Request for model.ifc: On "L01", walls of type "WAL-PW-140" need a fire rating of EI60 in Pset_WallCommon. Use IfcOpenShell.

First a look at what the model holds.

```python
import ifcopenshell
import ifcopenshell.util.element

model = ifcopenshell.open("model.ifc")
print(model.schema)
storey = next(s for s in model.by_type("IfcBuildingStorey") if s.Name == "L01")
walls = [e for e in ifcopenshell.util.element.get_decomposition(storey) if e.is_a("IfcWall")]
seen = {}
for e in walls:
    element_type = ifcopenshell.util.element.get_type(e)
    key = (element_type.Name if element_type != e and element_type else None, ifcopenshell.util.element.get_pset(e, "Pset_WallCommon", "FireRating"))
    seen[key] = seen.get(key, 0) + 1
for (name, value), count in sorted(seen.items(), key=str):
    print(count, "x", name, "|", value)
```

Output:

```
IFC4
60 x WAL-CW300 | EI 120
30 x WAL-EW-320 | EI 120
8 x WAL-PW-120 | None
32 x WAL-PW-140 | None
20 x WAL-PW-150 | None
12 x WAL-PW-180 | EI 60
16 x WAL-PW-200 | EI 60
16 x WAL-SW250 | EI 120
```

```python
import ifcopenshell
import ifcopenshell.api.pset
import ifcopenshell.util.element

model = ifcopenshell.open("model.ifc")

storey = next(s for s in model.by_type("IfcBuildingStorey") if s.Name == "L01")
walls = [e for e in ifcopenshell.util.element.get_decomposition(storey) if e.is_a("IfcWall")]

count = 0
for e in walls:
    element_type = ifcopenshell.util.element.get_type(e)
    if element_type in (None, e) or element_type.Name != "WAL-PW-140":
        continue
    # add_pset returns the element's existing set when there is one.
    pset = ifcopenshell.api.pset.add_pset(model, product=e, name="Pset_WallCommon")
    ifcopenshell.api.pset.edit_pset(model, pset=pset, properties={"FireRating": "EI60"})
    count += 1

print(count, "walls updated")

model.write("model_rev.ifc")
```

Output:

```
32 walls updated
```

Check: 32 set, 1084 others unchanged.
